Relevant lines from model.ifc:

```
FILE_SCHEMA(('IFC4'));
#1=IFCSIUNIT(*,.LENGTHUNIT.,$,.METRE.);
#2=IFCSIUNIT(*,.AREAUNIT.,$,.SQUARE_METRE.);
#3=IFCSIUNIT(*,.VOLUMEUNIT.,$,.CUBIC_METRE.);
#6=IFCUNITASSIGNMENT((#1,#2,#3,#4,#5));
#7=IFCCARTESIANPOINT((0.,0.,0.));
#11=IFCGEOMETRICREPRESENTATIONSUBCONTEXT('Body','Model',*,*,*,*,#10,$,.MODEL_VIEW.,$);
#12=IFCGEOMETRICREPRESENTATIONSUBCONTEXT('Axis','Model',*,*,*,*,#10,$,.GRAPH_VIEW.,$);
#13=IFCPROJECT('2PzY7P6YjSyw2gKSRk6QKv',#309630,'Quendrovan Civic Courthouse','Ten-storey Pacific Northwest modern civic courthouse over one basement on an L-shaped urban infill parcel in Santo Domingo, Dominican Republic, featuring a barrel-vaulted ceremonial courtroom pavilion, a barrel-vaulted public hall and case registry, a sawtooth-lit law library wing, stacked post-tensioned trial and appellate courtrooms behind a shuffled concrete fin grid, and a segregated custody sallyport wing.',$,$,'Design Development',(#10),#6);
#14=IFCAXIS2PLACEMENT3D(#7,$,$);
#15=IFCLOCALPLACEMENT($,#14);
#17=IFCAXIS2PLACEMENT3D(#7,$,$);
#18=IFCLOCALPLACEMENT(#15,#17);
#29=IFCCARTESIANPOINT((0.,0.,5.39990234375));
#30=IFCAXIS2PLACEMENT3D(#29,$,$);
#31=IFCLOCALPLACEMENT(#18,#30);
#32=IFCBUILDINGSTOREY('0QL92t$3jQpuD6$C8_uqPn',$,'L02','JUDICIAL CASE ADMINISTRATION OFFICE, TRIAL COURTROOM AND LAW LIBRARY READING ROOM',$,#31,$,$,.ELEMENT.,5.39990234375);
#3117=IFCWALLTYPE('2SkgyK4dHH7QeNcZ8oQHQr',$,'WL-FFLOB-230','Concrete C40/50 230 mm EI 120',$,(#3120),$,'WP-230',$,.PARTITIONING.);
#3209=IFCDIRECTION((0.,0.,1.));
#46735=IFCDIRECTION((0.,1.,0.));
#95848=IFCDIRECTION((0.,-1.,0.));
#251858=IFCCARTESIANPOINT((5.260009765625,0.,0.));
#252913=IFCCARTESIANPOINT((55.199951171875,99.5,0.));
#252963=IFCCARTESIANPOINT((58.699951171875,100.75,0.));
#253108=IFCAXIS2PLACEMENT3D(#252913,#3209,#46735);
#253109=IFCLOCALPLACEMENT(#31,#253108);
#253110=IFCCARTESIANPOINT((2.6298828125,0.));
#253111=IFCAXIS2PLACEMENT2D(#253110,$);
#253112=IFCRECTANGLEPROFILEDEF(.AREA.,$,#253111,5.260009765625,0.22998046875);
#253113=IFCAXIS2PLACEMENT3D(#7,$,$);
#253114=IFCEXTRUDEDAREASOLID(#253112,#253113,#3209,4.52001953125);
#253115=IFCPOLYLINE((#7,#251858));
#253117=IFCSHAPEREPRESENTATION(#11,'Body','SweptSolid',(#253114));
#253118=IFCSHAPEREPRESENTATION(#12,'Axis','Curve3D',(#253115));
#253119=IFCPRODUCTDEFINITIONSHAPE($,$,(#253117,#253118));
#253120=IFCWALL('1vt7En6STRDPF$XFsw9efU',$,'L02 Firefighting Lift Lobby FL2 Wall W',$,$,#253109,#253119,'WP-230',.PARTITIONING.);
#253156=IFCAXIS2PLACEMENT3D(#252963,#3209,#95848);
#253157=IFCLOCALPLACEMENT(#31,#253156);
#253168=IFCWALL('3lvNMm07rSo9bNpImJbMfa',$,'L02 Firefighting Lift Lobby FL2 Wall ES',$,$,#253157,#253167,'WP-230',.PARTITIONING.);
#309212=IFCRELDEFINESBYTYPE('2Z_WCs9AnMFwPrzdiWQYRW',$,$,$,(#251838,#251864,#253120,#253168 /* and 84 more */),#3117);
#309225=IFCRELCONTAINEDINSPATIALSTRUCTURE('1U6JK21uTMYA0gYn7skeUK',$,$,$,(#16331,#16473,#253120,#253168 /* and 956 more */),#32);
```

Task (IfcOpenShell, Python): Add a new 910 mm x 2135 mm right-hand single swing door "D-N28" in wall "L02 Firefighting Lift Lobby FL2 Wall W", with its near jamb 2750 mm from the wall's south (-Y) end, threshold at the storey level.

```python
import numpy as np
import ifcopenshell
import ifcopenshell.api.feature
import ifcopenshell.api.geometry
import ifcopenshell.api.root
import ifcopenshell.api.spatial
import ifcopenshell.geom
import ifcopenshell.util.element
import ifcopenshell.util.placement
import ifcopenshell.util.representation
import ifcopenshell.util.shape
import ifcopenshell.util.unit

model = ifcopenshell.open("model.ifc")
unit_scale = ifcopenshell.util.unit.calculate_unit_scale(model)
settings = ifcopenshell.geom.settings()


def volume(element):
    """Net volume in cubic metres, openings subtracted."""
    shape = ifcopenshell.geom.create_shape(settings, element)
    return ifcopenshell.util.shape.get_volume(shape.geometry)


wall = model.by_guid("1vt7En6STRDPF$XFsw9efU")
storey = ifcopenshell.util.element.get_container(wall, ifc_class="IfcBuildingStorey")
context = ifcopenshell.util.representation.get_context(model, "Model", "Body", "MODEL_VIEW")
before = volume(wall)

width, height, from_end, sill = 0.91, 2.135, 2.75, 0.0  # metres

# The wall runs along its own X axis, and the end named is its -X end.
wall_shape = ifcopenshell.geom.create_shape(settings, wall)
x, y, z = ifcopenshell.util.shape.get_vertices(wall_shape.geometry).T
start = x.min() + from_end
face, thickness = float(y.min()), float(y.max() - y.min())
wall_matrix = ifcopenshell.util.placement.get_local_placement(wall.ObjectPlacement)
level = ifcopenshell.util.placement.get_local_placement(storey.ObjectPlacement)[2, 3]


def in_wall(x, y):
    """Placement at x, y metres in the wall's axes, at sill height."""
    matrix = wall_matrix.copy()
    matrix[:, 3] = wall_matrix @ np.array([x / unit_scale, y / unit_scale, 0.0, 1.0])
    matrix[2, 3] = level + sill / unit_scale
    return matrix


# Opening: a box that overshoots both wall faces by 50 mm.
opening = ifcopenshell.api.root.create_entity(model, ifc_class="IfcOpeningElement", predefined_type="OPENING")
box = ifcopenshell.api.geometry.add_wall_representation(
    model, context=context, length=width, height=height, thickness=thickness + 0.1
)
ifcopenshell.api.geometry.assign_representation(model, product=opening, representation=box)
ifcopenshell.api.geometry.edit_object_placement(model, product=opening, matrix=in_wall(start, face - 0.05), is_si=False)
ifcopenshell.api.feature.add_feature(model, feature=opening, element=wall)

door = ifcopenshell.api.root.create_entity(model, ifc_class="IfcDoor", name="D-N28", predefined_type="DOOR")
door.OverallWidth, door.OverallHeight = width / unit_scale, height / unit_scale
door.OperationType = "SINGLE_SWING_RIGHT"
body = ifcopenshell.api.geometry.add_door_representation(
    model,
    context=context,
    overall_width=door.OverallWidth,
    overall_height=door.OverallHeight,
    operation_type="SINGLE_SWING_RIGHT",
    lining_properties={"LiningDepth": thickness / unit_scale, "ThresholdDepth": thickness / unit_scale},
)
ifcopenshell.api.geometry.assign_representation(model, product=door, representation=body)
ifcopenshell.api.spatial.assign_container(model, products=[door], relating_structure=storey)
ifcopenshell.api.feature.add_filling(model, opening=opening, element=door)

# The lining spans the wall, so the door starts at the wall face.
ifcopenshell.api.geometry.edit_object_placement(model, product=door, matrix=in_wall(start, face), is_si=False)

after = volume(wall)

print(f"wall volume {before:.3f} -> {after:.3f} m3")

model.write("model_rev.ifc")
```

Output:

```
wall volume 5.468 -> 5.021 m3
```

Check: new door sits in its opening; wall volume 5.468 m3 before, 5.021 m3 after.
